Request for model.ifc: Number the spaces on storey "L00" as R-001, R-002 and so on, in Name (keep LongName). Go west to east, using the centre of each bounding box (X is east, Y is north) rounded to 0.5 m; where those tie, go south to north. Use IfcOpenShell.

First a look at what the model holds.

```python
import ifcopenshell
import ifcopenshell.util.element
import ifcopenshell.util.placement

model = ifcopenshell.open("model.ifc")
print(model.schema)
storey = next(s for s in model.by_type("IfcBuildingStorey") if s.Name == "L00")
spaces = [e for e in ifcopenshell.util.element.get_decomposition(storey) if e.is_a("IfcSpace")]
for e in sorted(spaces, key=lambda e: e.id()):
    origin = ifcopenshell.util.placement.get_local_placement(e.ObjectPlacement)[:3, 3]
    print(e.id(), e.Name, e.LongName, origin.round(2) + 0.0, sep=" | ")
```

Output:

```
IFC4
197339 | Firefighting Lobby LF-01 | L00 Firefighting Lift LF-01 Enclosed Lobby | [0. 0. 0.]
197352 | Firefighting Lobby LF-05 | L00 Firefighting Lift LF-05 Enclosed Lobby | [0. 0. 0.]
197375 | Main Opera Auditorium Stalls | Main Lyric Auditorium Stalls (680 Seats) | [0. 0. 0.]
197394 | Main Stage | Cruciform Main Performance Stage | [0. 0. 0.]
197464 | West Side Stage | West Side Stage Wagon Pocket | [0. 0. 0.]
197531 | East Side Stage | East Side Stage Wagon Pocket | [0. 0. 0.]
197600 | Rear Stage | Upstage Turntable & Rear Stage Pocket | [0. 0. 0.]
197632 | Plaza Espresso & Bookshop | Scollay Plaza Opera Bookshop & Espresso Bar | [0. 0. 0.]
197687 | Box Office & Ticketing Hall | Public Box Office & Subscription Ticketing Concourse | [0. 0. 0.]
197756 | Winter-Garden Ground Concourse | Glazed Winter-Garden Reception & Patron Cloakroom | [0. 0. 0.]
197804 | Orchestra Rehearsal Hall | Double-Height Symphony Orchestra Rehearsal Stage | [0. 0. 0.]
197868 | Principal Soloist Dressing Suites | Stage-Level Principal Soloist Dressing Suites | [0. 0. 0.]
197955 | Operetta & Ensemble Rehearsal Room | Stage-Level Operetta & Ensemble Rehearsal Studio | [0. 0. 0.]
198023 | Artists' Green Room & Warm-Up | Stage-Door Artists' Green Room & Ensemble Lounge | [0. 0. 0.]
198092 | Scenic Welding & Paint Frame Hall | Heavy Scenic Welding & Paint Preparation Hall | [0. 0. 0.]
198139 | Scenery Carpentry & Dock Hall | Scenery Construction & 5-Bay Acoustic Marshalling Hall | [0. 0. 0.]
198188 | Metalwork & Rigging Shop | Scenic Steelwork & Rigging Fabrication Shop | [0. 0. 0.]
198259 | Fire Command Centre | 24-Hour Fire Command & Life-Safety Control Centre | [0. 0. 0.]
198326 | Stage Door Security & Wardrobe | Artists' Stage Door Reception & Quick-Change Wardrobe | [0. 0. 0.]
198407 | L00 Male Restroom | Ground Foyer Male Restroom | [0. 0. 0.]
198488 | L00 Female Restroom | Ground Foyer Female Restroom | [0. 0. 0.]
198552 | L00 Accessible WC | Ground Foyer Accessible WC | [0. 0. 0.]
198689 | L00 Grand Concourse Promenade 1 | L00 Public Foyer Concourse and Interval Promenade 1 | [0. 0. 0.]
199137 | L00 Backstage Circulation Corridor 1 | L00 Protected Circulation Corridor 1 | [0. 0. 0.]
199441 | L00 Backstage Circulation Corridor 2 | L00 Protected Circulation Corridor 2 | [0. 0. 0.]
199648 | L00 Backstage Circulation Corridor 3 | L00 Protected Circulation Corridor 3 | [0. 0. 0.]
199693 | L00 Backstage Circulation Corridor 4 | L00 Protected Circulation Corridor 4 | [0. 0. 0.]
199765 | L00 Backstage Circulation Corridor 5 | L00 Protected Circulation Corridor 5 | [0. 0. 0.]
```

```python
import ifcopenshell
import ifcopenshell.geom
import ifcopenshell.util.element
import ifcopenshell.util.shape

model = ifcopenshell.open("model.ifc")
settings = ifcopenshell.geom.settings()
settings.set("use-world-coords", True)


def centre(element):
    shape = ifcopenshell.geom.create_shape(settings, element)
    return ifcopenshell.util.shape.get_bbox_centroid(shape.geometry)


storey = next(s for s in model.by_type("IfcBuildingStorey") if s.Name == "L00")
spaces = [e for e in ifcopenshell.util.element.get_decomposition(storey) if e.is_a("IfcSpace")]

# Insertion points can sit at a corner or the storey origin, so sort by the geometry (in metres).
centres = {e: centre(e) for e in spaces}
spaces.sort(key=lambda e: (round(centres[e][0] / 0.5), centres[e][1]))

for i, e in enumerate(spaces, start=1):
    number = f"R-0{i:02d}"
    e.Name = number
    print(e.id(), number)

model.write("model_v2.ifc")
```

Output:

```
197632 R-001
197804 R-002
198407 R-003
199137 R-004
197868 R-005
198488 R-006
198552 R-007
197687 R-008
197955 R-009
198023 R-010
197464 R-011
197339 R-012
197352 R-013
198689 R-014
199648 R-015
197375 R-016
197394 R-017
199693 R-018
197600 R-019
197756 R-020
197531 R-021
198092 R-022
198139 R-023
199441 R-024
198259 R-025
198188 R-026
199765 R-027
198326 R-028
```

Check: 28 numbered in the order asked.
